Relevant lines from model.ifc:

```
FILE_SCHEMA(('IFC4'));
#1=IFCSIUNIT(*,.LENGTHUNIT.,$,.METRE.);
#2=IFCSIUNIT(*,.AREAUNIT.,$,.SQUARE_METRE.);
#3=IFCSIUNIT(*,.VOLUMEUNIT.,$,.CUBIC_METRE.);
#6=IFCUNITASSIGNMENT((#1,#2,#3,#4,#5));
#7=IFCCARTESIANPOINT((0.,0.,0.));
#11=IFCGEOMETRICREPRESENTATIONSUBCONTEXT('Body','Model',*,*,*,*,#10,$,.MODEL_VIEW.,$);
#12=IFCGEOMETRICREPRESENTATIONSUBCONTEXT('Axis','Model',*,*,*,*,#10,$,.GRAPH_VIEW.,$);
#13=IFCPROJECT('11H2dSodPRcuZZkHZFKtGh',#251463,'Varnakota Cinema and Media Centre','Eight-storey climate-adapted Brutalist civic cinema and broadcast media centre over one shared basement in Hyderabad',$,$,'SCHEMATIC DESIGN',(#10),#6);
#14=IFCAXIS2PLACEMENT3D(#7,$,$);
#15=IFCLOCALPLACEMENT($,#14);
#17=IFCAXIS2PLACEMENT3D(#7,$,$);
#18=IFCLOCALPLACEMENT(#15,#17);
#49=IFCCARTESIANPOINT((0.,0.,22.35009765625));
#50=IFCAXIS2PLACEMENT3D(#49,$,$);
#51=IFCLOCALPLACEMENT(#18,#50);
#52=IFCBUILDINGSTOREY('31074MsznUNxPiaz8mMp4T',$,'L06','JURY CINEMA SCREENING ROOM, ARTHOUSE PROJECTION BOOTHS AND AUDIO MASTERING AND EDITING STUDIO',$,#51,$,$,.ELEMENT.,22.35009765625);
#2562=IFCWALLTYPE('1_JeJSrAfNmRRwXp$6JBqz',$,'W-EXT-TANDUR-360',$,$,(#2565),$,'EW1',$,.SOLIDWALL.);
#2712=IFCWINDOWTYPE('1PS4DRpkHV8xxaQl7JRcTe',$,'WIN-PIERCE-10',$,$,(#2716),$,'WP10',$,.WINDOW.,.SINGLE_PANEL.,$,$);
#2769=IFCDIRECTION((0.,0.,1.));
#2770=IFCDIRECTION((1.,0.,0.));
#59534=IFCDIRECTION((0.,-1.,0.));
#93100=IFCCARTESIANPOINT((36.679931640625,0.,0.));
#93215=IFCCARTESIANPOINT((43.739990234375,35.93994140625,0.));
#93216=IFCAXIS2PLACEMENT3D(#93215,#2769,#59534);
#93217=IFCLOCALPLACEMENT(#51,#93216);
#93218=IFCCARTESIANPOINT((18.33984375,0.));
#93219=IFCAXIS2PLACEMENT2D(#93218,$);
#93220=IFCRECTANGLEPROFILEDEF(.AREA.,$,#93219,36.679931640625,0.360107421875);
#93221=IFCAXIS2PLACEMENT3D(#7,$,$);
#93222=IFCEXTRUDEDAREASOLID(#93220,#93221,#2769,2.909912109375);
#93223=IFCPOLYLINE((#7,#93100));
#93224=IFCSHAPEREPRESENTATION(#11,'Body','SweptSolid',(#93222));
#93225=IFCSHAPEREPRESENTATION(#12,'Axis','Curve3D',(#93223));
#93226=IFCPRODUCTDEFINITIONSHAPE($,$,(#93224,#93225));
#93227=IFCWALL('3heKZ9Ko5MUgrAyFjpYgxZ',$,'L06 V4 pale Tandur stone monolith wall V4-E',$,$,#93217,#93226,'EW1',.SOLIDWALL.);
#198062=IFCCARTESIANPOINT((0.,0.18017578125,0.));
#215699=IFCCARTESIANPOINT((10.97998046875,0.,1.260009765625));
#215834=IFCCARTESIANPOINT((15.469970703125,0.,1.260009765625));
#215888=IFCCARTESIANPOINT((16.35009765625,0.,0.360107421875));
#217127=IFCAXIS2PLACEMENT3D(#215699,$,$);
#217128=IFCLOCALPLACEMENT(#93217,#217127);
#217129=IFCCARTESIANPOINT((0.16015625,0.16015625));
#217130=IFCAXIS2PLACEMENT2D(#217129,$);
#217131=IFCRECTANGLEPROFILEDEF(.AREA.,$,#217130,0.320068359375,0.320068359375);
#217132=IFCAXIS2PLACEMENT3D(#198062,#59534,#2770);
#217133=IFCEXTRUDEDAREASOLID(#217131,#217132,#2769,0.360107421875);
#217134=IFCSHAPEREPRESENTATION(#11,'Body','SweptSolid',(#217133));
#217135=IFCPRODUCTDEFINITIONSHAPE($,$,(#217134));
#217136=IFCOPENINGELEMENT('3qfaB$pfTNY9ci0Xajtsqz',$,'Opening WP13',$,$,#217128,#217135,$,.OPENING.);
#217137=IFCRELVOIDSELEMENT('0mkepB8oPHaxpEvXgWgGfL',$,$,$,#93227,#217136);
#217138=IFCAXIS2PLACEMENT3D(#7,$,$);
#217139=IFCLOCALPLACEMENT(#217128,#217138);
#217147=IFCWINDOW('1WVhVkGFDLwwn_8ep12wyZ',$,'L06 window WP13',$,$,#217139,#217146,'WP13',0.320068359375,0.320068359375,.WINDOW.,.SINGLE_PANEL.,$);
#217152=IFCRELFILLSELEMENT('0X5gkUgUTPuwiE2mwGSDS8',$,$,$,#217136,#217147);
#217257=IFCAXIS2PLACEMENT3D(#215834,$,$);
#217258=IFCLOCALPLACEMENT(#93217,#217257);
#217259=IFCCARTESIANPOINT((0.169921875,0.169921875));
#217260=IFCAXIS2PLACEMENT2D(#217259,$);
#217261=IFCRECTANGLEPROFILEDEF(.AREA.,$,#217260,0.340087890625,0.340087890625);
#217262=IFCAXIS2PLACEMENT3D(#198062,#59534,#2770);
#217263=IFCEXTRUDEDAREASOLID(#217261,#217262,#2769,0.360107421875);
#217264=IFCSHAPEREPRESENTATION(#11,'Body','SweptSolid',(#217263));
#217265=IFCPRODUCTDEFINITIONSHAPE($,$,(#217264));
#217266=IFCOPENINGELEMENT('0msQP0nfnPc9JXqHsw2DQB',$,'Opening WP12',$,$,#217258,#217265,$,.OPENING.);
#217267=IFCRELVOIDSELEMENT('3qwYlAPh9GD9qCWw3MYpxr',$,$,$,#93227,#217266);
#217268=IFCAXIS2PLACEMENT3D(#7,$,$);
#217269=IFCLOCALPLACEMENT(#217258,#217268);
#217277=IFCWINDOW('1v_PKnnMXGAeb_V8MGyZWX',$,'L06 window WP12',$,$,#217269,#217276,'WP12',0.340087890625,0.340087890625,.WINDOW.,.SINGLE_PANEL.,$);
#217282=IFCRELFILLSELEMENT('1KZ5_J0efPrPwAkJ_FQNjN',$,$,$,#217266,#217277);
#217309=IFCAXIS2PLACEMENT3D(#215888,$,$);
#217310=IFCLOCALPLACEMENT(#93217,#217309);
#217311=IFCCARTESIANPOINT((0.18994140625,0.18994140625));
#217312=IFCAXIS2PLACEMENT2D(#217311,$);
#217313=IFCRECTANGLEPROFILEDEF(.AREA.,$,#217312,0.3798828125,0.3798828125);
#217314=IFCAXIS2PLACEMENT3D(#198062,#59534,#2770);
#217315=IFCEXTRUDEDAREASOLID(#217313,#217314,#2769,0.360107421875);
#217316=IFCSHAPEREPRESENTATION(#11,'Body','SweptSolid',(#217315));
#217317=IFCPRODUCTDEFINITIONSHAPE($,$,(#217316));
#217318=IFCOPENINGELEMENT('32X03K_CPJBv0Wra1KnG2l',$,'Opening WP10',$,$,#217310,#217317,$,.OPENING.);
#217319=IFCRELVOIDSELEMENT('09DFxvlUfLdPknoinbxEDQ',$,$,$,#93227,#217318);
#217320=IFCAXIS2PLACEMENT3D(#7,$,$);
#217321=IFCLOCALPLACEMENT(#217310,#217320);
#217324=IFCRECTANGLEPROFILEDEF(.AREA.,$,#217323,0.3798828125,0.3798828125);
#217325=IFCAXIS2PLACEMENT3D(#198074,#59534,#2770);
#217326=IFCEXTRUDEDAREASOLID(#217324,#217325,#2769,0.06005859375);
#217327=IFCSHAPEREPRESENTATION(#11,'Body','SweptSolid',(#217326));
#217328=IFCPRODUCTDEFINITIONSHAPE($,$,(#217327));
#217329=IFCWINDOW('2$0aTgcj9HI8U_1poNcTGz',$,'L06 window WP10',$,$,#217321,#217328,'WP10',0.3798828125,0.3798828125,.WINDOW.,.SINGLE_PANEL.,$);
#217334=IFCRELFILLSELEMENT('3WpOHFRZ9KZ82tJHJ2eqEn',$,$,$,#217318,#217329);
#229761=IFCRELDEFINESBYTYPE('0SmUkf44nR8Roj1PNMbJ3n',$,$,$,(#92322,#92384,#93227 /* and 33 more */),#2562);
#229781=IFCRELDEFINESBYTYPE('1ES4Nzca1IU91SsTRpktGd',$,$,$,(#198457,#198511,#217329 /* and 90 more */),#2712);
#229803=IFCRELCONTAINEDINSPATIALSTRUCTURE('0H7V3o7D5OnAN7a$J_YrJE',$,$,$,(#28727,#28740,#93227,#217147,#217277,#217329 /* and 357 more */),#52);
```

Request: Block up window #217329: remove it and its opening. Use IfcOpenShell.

```python
import ifcopenshell
import ifcopenshell.api.feature
import ifcopenshell.api.root
import ifcopenshell.geom
import ifcopenshell.util.shape

model = ifcopenshell.open("model.ifc")
settings = ifcopenshell.geom.settings()


def volume(element):
    """Net volume in cubic metres, openings subtracted."""
    shape = ifcopenshell.geom.create_shape(settings, element)
    return ifcopenshell.util.shape.get_volume(shape.geometry)


window = model.by_guid("2$0aTgcj9HI8U_1poNcTGz")
opening = window.FillsVoids[0].RelatingOpeningElement
wall = opening.VoidsElements[0].RelatingBuildingElement
before = volume(wall)

ifcopenshell.api.root.remove_product(model, product=window)
ifcopenshell.api.feature.remove_feature(model, feature=opening)

after = volume(wall)

print(f"wall volume {before:.3f} -> {after:.3f} m3")

model.write("model_rev.ifc")
```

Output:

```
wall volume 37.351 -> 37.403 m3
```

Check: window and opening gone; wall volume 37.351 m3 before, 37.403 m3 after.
